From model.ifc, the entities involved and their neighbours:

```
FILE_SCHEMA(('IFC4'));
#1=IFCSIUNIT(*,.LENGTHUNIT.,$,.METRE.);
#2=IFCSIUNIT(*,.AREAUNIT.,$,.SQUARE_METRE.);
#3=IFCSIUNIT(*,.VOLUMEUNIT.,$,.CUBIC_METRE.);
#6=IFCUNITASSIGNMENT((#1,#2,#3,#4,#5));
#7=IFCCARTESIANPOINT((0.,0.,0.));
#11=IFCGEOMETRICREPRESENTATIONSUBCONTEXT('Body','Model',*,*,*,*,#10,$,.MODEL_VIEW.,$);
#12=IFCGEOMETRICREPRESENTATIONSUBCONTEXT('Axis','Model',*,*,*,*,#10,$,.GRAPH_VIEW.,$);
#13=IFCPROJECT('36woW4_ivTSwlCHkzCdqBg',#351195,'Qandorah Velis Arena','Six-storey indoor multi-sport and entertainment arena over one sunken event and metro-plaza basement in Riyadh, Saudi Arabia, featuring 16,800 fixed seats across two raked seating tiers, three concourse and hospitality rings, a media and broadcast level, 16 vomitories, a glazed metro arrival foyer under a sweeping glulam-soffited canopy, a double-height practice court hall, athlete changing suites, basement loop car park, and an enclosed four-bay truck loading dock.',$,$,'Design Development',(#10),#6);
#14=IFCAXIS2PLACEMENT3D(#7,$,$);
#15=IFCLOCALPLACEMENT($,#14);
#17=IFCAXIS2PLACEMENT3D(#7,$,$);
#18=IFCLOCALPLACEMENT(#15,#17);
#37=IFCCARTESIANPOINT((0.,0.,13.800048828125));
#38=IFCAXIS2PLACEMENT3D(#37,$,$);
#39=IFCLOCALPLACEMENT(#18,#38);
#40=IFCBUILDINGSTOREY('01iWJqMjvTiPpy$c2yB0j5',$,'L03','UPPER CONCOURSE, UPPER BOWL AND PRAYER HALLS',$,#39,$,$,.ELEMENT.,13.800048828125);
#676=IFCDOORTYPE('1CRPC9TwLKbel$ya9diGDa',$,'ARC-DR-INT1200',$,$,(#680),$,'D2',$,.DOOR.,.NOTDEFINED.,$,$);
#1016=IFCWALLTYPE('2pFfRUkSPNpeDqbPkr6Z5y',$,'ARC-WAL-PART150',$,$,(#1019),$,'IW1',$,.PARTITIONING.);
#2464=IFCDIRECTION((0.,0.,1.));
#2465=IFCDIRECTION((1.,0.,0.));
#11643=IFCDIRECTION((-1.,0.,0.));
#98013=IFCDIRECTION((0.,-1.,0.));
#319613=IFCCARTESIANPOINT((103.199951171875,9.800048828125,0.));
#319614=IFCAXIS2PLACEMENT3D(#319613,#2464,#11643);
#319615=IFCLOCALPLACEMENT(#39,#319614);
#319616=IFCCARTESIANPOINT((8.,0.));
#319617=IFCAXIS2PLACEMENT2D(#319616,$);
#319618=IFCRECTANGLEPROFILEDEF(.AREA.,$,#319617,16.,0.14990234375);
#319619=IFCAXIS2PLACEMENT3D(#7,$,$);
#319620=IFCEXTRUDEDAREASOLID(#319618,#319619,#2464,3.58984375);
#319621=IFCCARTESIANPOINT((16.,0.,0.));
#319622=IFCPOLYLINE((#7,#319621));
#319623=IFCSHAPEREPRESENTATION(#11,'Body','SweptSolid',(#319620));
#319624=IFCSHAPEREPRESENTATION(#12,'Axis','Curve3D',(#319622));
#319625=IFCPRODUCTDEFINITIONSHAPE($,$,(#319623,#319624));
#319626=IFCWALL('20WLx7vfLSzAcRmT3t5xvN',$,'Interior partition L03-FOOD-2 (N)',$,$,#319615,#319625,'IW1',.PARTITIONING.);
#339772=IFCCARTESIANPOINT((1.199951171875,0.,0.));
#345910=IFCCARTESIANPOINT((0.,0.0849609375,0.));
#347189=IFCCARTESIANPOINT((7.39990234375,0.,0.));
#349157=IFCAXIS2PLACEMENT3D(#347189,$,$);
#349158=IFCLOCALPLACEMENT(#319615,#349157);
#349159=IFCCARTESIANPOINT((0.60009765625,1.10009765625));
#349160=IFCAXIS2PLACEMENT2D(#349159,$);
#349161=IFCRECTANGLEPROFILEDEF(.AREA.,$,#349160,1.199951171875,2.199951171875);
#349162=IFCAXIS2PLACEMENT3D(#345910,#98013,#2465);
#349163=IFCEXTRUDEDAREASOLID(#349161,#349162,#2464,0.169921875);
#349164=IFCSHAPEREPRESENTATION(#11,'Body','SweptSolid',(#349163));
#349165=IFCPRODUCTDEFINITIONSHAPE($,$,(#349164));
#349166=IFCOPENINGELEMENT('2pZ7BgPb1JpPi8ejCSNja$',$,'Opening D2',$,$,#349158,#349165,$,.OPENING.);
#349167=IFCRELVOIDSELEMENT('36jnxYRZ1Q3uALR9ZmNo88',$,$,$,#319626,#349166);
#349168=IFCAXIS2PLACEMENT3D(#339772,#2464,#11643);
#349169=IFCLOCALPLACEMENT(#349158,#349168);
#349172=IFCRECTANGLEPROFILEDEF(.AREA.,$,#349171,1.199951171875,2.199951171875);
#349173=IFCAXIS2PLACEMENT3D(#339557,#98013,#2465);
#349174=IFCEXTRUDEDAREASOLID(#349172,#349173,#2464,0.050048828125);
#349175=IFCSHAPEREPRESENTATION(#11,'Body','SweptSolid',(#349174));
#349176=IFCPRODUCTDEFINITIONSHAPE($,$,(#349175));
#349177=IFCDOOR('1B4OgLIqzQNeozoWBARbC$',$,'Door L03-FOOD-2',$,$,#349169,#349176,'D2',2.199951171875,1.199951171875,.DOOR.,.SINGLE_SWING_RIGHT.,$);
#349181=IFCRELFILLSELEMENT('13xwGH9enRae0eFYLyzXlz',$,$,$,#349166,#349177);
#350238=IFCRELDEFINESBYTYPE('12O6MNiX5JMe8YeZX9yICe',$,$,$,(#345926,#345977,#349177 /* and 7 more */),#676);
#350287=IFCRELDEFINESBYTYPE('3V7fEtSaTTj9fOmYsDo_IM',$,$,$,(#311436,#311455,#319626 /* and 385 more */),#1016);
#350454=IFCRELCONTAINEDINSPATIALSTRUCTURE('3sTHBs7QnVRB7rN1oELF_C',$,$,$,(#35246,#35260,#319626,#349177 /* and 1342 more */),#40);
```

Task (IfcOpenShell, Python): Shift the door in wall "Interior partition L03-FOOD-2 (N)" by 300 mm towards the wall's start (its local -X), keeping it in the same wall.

```python
import ifcopenshell
import ifcopenshell.api.geometry
import ifcopenshell.util.placement
import ifcopenshell.util.unit

model = ifcopenshell.open("model.ifc")
unit_scale = ifcopenshell.util.unit.calculate_unit_scale(model)

door = model.by_id(349177)
opening = door.FillsVoids[0].RelatingOpeningElement
wall = opening.VoidsElements[0].RelatingBuildingElement

wall_matrix = ifcopenshell.util.placement.get_local_placement(wall.ObjectPlacement)
shift = wall_matrix[:3, 0] * -0.3 / unit_scale
before = ifcopenshell.util.placement.get_local_placement(door.ObjectPlacement)[:3, 3].copy()

# The door is placed relative to its opening, so it follows when the opening moves.
matrix = ifcopenshell.util.placement.get_local_placement(opening.ObjectPlacement)
matrix[:3, 3] += shift
ifcopenshell.api.geometry.edit_object_placement(
    model, product=opening, matrix=matrix, is_si=False, should_transform_children=True
)

after = ifcopenshell.util.placement.get_local_placement(door.ObjectPlacement)[:3, 3]
print("door moved by", (after - before).round(3) + 0.0)

model.write("model_rev.ifc")
```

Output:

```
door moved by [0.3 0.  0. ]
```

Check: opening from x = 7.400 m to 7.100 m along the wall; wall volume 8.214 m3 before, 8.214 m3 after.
